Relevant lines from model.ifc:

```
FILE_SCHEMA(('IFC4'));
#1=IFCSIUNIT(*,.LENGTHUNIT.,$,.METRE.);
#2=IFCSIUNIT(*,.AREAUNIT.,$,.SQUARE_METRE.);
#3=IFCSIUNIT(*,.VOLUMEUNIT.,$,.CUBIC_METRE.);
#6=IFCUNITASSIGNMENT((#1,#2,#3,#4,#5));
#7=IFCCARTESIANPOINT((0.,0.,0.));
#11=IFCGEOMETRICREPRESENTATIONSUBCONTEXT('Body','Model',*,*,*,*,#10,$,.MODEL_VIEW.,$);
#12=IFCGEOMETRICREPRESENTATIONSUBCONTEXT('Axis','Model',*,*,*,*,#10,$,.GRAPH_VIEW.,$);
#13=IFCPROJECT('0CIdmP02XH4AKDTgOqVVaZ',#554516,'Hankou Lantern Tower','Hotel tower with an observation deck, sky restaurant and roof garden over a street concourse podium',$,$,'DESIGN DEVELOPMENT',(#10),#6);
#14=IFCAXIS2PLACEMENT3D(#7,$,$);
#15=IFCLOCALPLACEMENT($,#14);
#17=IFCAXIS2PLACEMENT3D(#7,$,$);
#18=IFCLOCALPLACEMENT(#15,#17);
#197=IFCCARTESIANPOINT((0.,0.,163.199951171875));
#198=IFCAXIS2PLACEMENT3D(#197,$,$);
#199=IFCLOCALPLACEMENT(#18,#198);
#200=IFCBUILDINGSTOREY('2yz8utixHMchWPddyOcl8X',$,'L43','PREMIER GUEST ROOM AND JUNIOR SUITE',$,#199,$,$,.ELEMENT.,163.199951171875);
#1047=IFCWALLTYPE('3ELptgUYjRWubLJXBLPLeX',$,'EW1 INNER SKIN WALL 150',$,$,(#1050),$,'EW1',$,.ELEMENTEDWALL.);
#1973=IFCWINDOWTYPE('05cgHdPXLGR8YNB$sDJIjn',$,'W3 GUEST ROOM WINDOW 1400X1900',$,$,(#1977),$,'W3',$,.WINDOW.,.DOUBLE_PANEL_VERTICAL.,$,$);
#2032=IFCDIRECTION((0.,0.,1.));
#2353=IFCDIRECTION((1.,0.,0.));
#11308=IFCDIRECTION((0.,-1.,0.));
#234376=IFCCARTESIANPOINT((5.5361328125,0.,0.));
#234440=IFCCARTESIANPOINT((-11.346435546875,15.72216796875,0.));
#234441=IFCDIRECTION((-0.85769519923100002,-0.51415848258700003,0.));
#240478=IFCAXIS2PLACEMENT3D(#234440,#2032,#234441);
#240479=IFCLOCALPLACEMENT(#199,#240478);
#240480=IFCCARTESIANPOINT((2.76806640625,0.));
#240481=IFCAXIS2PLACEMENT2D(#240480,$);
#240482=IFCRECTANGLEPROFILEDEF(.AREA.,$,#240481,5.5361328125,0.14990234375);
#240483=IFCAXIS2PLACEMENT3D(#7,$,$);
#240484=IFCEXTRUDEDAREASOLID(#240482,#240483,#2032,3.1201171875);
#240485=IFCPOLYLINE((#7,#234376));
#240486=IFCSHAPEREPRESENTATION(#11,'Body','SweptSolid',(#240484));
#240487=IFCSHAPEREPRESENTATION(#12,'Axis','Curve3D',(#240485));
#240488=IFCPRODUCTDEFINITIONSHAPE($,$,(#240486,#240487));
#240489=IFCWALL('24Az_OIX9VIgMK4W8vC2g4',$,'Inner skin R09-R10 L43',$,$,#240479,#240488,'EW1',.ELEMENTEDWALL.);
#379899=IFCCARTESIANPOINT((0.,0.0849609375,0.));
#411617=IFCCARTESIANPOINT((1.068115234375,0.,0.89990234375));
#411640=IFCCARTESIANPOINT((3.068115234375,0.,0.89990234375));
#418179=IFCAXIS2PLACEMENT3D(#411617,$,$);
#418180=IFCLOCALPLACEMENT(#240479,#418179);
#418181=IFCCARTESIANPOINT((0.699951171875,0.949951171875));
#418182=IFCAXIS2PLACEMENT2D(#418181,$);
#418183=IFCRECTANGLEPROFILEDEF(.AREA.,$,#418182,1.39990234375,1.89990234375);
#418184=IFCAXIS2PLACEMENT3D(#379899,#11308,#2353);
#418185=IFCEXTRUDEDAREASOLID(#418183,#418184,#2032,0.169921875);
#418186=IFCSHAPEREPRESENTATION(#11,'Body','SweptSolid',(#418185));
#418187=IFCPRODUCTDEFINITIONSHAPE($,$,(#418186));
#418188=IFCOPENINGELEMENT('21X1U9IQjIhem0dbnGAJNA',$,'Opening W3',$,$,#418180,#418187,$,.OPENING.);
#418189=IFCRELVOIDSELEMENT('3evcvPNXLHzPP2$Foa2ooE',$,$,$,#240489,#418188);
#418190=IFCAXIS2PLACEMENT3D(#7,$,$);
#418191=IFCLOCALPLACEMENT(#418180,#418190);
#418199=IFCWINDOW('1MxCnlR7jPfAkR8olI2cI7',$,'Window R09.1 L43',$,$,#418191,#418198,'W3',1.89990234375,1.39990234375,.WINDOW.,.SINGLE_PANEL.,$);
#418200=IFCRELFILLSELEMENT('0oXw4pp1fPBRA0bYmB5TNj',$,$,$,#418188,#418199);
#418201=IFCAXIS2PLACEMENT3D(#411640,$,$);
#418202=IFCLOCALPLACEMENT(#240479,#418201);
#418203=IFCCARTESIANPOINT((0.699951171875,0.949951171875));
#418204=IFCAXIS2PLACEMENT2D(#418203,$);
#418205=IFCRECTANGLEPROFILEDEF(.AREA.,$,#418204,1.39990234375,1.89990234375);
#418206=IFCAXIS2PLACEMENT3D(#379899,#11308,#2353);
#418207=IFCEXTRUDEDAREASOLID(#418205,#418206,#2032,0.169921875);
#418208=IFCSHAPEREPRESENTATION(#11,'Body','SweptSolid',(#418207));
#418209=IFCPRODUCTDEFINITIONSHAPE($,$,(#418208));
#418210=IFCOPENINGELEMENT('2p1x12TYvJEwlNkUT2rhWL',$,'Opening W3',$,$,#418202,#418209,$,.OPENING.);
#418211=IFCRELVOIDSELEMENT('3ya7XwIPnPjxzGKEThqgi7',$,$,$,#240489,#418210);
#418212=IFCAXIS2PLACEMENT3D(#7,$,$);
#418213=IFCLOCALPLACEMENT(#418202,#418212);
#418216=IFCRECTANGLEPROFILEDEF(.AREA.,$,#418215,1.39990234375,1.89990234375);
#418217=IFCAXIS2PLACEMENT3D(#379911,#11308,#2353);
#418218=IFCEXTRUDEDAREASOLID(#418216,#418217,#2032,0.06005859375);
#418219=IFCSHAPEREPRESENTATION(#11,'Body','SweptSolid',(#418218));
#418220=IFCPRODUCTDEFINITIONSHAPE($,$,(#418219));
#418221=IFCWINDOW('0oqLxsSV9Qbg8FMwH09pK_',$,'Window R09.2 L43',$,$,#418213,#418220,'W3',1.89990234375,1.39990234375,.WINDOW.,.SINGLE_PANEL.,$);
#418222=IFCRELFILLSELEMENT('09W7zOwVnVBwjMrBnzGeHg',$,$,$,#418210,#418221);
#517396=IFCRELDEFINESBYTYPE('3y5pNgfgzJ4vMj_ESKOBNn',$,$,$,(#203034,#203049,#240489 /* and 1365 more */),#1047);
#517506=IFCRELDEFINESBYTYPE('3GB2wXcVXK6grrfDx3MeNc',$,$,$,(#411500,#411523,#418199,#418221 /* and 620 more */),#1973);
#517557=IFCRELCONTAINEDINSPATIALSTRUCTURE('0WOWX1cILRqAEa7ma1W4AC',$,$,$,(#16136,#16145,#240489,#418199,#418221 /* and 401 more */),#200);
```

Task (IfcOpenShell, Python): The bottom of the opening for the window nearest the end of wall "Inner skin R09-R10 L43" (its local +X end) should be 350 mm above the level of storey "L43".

```python
import numpy as np
import ifcopenshell
import ifcopenshell.api.geometry
import ifcopenshell.geom
import ifcopenshell.util.element
import ifcopenshell.util.placement
import ifcopenshell.util.shape
import ifcopenshell.util.unit

model = ifcopenshell.open("model.ifc")
unit_scale = ifcopenshell.util.unit.calculate_unit_scale(model)

window = model.by_id(418221)
opening = window.FillsVoids[0].RelatingOpeningElement
storey = ifcopenshell.util.element.get_container(window, ifc_class="IfcBuildingStorey")
level = ifcopenshell.util.placement.get_local_placement(storey.ObjectPlacement)[2, 3]

# The opening's origin need not be at the sill, so measure its lowest point.
shape = ifcopenshell.geom.create_shape(ifcopenshell.geom.settings(), opening)
bottom = ifcopenshell.util.shape.get_shape_bottom_elevation(shape, shape.geometry) / unit_scale
dz = level + 0.35 / unit_scale - bottom

shift = np.array([0.0, 0.0, dz])
# The window is placed relative to its opening, so it follows when the opening moves.
matrix = ifcopenshell.util.placement.get_local_placement(opening.ObjectPlacement)
matrix[:3, 3] += shift
ifcopenshell.api.geometry.edit_object_placement(
    model, product=opening, matrix=matrix, is_si=False, should_transform_children=True
)

print(f"moved by {dz * unit_scale:+.3f} m")

model.write("model-out.ifc")
```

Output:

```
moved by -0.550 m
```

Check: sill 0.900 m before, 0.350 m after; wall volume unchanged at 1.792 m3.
